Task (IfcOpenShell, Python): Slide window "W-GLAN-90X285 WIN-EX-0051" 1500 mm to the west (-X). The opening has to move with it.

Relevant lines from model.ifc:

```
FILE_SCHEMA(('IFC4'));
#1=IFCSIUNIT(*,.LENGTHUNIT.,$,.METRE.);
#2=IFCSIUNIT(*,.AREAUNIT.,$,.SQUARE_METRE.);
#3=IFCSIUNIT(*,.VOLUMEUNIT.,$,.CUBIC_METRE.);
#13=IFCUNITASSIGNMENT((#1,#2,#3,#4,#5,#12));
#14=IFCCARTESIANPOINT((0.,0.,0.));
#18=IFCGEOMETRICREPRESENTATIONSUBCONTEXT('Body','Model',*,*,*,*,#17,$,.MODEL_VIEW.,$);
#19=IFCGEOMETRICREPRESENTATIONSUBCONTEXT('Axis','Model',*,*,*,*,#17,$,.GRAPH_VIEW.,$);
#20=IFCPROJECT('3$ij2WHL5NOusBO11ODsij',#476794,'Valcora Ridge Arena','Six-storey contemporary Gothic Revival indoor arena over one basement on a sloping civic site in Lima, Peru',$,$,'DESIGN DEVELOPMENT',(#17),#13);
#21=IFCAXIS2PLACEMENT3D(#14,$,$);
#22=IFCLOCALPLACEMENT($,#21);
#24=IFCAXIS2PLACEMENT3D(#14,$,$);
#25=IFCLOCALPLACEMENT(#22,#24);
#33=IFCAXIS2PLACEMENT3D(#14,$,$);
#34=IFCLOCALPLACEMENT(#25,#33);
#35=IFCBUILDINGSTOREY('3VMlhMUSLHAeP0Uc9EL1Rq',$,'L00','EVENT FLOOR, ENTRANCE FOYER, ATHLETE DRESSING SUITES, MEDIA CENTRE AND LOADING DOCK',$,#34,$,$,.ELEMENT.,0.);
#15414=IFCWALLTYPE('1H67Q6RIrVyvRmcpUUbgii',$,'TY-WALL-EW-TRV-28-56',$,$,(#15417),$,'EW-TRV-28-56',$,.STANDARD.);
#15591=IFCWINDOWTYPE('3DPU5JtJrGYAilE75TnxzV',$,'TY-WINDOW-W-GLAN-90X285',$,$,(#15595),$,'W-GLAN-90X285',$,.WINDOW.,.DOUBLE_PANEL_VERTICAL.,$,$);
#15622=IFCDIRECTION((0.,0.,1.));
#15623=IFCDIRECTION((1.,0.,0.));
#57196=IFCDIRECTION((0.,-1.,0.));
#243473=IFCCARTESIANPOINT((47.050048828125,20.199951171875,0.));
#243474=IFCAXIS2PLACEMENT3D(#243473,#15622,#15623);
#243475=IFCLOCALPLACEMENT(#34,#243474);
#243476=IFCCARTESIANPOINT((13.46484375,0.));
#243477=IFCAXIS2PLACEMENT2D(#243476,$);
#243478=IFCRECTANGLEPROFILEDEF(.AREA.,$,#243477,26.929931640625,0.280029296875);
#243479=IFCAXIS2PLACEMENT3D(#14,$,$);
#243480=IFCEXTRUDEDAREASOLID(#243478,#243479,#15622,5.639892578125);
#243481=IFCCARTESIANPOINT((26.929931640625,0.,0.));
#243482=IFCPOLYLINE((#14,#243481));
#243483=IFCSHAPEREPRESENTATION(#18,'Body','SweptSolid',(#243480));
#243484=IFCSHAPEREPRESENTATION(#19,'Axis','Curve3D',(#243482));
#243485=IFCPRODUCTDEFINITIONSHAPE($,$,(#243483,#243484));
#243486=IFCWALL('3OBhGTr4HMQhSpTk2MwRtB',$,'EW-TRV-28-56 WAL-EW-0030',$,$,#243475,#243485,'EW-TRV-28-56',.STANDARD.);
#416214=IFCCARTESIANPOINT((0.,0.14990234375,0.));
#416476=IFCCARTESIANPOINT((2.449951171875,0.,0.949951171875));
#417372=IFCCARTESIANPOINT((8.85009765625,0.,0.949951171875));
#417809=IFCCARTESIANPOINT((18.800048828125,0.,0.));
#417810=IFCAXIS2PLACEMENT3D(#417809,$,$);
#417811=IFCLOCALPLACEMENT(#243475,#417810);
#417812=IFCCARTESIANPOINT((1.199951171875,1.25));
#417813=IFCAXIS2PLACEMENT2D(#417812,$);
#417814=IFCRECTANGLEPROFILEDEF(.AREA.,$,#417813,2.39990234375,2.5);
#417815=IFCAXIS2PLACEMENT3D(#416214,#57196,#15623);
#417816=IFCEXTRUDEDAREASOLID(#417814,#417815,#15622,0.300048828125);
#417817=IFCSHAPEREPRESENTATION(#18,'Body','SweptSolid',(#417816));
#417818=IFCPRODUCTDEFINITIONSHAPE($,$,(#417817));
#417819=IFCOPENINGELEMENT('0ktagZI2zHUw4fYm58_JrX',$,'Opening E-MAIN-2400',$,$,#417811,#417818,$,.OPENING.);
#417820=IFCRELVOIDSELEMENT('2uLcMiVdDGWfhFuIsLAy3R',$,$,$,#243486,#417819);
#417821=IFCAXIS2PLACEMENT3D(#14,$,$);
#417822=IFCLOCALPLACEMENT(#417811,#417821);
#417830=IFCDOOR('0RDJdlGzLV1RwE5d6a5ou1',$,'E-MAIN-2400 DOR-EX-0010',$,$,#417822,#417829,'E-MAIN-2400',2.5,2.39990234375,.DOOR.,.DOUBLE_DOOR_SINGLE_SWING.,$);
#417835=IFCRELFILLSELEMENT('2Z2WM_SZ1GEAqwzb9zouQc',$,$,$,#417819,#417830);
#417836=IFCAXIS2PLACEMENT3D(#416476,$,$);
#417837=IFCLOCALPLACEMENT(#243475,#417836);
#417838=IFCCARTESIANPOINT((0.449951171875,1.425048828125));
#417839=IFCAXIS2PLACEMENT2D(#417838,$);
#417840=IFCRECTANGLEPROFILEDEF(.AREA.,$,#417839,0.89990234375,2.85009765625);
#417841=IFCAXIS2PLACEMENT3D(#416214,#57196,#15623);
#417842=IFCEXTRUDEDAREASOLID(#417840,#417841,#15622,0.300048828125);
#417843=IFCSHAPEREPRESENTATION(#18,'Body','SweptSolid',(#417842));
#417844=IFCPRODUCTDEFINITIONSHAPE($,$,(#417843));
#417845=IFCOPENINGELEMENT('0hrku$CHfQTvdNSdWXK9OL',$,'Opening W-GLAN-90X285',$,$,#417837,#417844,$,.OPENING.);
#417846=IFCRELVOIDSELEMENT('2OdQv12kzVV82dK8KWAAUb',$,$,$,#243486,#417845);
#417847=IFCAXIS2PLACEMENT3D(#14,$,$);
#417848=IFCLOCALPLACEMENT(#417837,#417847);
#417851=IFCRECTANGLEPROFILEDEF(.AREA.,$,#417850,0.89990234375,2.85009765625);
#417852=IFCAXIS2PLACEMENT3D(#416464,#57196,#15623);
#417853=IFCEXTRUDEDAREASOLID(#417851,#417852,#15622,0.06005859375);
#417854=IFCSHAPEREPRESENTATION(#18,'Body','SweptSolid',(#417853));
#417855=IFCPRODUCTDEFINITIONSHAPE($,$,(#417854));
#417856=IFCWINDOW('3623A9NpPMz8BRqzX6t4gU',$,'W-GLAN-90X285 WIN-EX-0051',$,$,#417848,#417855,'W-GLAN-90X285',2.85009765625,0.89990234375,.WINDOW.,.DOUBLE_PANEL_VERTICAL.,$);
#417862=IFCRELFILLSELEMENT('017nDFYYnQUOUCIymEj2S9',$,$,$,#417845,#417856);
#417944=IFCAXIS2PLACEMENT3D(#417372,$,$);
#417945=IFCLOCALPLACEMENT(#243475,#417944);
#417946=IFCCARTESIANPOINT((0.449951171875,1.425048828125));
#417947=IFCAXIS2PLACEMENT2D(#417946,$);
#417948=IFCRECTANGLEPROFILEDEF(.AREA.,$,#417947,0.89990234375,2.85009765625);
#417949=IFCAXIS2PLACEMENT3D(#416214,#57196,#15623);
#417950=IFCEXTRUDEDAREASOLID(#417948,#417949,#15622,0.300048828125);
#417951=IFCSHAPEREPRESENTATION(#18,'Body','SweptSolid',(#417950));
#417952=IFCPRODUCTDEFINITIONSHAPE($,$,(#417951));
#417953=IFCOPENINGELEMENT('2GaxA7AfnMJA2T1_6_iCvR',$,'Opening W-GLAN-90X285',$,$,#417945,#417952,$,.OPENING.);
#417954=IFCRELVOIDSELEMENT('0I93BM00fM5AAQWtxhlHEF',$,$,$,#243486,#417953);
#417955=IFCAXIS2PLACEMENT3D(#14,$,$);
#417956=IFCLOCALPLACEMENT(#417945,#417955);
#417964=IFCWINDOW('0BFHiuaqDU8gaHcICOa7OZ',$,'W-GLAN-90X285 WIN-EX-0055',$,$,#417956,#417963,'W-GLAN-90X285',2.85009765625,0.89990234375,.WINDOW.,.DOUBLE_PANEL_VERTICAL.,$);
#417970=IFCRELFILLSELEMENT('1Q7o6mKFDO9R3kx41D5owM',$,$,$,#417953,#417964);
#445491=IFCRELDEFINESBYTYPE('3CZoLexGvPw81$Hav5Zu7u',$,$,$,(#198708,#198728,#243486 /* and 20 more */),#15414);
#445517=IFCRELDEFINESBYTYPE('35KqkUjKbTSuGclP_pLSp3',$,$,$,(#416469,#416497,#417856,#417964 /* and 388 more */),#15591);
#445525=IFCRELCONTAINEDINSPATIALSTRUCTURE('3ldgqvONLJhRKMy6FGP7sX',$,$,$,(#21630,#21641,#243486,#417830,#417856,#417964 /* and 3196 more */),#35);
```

```python
import ifcopenshell
import ifcopenshell.api.geometry
import ifcopenshell.util.placement
import ifcopenshell.util.unit

model = ifcopenshell.open("model.ifc")
unit_scale = ifcopenshell.util.unit.calculate_unit_scale(model)

window = model.by_guid("3623A9NpPMz8BRqzX6t4gU")
opening = window.FillsVoids[0].RelatingOpeningElement
wall = opening.VoidsElements[0].RelatingBuildingElement

wall_matrix = ifcopenshell.util.placement.get_local_placement(wall.ObjectPlacement)
shift = wall_matrix[:3, 0] * -1.5 / unit_scale
before = ifcopenshell.util.placement.get_local_placement(window.ObjectPlacement)[:3, 3].copy()

# The window is placed relative to its opening, so it follows when the opening moves.
matrix = ifcopenshell.util.placement.get_local_placement(opening.ObjectPlacement)
matrix[:3, 3] += shift
ifcopenshell.api.geometry.edit_object_placement(
    model, product=opening, matrix=matrix, is_si=False, should_transform_children=True
)

after = ifcopenshell.util.placement.get_local_placement(window.ObjectPlacement)[:3, 3]
print("window moved by", (after - before).round(3) + 0.0)

model.write("model_edited.ifc")
```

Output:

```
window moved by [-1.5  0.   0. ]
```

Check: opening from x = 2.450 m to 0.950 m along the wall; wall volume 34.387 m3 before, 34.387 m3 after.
